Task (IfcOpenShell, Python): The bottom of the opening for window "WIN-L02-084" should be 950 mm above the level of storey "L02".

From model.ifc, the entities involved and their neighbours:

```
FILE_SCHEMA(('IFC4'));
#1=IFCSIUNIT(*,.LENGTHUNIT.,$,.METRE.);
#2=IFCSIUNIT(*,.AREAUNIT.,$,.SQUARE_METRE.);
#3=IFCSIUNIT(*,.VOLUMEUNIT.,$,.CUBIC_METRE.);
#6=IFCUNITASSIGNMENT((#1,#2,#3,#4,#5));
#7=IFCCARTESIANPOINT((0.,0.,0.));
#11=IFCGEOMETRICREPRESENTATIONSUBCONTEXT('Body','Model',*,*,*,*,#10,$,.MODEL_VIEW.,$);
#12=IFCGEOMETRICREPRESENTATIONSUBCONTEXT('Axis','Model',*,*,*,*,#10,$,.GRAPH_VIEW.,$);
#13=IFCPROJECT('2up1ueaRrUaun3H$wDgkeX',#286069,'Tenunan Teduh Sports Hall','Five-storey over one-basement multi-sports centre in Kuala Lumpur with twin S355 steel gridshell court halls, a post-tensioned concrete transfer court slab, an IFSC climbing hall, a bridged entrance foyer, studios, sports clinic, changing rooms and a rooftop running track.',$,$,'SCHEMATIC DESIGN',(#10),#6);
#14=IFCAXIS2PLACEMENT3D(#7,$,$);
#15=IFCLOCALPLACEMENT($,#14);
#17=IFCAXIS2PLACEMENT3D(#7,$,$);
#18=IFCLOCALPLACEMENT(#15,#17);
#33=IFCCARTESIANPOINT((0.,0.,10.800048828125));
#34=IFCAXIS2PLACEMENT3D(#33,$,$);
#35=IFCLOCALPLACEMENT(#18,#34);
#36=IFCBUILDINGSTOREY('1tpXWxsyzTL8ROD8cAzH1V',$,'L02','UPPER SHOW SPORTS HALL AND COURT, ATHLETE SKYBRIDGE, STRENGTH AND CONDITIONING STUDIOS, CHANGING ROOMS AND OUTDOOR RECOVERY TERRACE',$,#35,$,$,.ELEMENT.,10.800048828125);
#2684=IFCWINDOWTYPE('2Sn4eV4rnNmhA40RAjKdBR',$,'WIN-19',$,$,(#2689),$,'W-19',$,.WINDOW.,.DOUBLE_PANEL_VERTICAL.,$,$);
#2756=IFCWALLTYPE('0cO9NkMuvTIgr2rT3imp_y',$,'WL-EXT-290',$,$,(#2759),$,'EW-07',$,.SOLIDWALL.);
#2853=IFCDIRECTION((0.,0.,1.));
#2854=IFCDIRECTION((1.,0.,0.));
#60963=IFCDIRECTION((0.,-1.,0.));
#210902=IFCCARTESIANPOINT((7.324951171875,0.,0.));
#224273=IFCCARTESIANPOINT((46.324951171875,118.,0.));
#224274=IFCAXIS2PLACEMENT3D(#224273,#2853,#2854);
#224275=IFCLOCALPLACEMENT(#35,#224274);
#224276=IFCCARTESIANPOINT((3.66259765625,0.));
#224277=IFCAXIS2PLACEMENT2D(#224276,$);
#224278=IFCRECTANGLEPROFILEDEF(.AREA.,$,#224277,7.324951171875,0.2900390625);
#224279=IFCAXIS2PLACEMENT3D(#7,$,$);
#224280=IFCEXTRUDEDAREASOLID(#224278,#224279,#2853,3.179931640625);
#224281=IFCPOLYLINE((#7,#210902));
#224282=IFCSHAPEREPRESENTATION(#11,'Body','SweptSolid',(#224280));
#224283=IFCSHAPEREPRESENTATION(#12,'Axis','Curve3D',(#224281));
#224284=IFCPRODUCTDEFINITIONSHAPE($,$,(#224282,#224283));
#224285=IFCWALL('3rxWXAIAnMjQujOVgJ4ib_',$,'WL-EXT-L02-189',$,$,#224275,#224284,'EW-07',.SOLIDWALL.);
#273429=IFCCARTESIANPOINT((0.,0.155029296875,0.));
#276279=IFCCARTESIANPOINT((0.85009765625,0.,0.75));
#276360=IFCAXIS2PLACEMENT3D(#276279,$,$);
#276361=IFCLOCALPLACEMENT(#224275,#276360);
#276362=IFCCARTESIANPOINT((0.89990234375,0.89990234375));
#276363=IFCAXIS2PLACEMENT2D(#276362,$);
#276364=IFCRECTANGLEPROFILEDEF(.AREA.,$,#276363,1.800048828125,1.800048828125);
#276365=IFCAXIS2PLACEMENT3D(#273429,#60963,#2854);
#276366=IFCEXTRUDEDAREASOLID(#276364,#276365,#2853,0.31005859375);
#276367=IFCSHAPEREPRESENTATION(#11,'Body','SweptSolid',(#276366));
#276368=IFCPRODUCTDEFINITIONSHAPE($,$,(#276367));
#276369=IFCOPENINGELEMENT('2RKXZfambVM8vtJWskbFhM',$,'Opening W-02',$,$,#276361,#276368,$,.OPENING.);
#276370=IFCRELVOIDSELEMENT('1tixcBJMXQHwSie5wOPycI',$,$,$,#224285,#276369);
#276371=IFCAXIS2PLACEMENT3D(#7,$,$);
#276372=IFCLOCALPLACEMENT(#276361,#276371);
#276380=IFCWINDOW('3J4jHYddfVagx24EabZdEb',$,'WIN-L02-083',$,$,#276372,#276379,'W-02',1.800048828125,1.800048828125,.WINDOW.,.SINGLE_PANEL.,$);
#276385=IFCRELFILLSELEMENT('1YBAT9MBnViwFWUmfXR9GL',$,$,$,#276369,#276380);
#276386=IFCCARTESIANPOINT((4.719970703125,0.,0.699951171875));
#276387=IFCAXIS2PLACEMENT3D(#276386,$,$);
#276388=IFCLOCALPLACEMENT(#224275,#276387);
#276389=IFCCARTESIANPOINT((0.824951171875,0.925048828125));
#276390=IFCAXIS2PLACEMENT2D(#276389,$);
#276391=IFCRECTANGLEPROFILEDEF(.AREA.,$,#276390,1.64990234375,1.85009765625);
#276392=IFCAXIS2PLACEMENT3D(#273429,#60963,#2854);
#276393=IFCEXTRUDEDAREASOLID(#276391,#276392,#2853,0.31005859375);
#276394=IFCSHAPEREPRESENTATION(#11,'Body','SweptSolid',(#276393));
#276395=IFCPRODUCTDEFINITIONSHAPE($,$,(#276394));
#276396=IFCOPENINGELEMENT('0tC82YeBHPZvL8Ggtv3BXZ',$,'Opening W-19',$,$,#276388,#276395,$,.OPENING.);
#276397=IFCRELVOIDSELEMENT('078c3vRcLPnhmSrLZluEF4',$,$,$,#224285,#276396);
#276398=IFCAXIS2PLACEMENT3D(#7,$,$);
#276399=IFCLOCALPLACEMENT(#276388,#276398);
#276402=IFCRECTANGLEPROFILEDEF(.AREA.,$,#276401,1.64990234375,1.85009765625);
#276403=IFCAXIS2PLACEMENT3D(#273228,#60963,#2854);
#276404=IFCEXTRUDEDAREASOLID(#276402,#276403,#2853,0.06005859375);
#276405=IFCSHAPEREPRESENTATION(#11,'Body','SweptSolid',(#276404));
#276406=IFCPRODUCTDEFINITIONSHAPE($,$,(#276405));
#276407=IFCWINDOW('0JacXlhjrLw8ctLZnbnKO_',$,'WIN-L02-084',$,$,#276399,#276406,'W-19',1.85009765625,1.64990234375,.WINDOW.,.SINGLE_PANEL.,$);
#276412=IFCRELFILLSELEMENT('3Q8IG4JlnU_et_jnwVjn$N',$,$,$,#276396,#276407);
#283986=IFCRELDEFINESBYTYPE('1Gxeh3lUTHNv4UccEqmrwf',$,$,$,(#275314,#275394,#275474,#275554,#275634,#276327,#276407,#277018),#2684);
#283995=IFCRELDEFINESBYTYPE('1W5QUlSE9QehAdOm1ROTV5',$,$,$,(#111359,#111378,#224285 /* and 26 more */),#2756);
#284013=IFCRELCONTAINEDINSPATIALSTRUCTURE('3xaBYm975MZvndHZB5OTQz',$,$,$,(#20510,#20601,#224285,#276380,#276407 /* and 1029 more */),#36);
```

```python
import numpy as np
import ifcopenshell
import ifcopenshell.api.geometry
import ifcopenshell.geom
import ifcopenshell.util.element
import ifcopenshell.util.placement
import ifcopenshell.util.shape
import ifcopenshell.util.unit

model = ifcopenshell.open("model.ifc")
unit_scale = ifcopenshell.util.unit.calculate_unit_scale(model)

window = model.by_guid("0JacXlhjrLw8ctLZnbnKO_")
opening = window.FillsVoids[0].RelatingOpeningElement
storey = ifcopenshell.util.element.get_container(window, ifc_class="IfcBuildingStorey")
level = ifcopenshell.util.placement.get_local_placement(storey.ObjectPlacement)[2, 3]

# The opening's origin need not be at the sill, so measure its lowest point.
shape = ifcopenshell.geom.create_shape(ifcopenshell.geom.settings(), opening)
bottom = ifcopenshell.util.shape.get_shape_bottom_elevation(shape, shape.geometry) / unit_scale
dz = level + 0.95 - bottom

shift = np.array([0.0, 0.0, dz])
# The window is placed relative to its opening, so it follows when the opening moves.
matrix = ifcopenshell.util.placement.get_local_placement(opening.ObjectPlacement)
matrix[:3, 3] += shift
ifcopenshell.api.geometry.edit_object_placement(
    model, product=opening, matrix=matrix, is_si=False, should_transform_children=True
)

print(f"moved by {dz * unit_scale:+.3f} m")

model.write("model_v2.ifc")
```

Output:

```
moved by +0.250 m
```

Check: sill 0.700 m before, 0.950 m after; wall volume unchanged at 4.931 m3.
